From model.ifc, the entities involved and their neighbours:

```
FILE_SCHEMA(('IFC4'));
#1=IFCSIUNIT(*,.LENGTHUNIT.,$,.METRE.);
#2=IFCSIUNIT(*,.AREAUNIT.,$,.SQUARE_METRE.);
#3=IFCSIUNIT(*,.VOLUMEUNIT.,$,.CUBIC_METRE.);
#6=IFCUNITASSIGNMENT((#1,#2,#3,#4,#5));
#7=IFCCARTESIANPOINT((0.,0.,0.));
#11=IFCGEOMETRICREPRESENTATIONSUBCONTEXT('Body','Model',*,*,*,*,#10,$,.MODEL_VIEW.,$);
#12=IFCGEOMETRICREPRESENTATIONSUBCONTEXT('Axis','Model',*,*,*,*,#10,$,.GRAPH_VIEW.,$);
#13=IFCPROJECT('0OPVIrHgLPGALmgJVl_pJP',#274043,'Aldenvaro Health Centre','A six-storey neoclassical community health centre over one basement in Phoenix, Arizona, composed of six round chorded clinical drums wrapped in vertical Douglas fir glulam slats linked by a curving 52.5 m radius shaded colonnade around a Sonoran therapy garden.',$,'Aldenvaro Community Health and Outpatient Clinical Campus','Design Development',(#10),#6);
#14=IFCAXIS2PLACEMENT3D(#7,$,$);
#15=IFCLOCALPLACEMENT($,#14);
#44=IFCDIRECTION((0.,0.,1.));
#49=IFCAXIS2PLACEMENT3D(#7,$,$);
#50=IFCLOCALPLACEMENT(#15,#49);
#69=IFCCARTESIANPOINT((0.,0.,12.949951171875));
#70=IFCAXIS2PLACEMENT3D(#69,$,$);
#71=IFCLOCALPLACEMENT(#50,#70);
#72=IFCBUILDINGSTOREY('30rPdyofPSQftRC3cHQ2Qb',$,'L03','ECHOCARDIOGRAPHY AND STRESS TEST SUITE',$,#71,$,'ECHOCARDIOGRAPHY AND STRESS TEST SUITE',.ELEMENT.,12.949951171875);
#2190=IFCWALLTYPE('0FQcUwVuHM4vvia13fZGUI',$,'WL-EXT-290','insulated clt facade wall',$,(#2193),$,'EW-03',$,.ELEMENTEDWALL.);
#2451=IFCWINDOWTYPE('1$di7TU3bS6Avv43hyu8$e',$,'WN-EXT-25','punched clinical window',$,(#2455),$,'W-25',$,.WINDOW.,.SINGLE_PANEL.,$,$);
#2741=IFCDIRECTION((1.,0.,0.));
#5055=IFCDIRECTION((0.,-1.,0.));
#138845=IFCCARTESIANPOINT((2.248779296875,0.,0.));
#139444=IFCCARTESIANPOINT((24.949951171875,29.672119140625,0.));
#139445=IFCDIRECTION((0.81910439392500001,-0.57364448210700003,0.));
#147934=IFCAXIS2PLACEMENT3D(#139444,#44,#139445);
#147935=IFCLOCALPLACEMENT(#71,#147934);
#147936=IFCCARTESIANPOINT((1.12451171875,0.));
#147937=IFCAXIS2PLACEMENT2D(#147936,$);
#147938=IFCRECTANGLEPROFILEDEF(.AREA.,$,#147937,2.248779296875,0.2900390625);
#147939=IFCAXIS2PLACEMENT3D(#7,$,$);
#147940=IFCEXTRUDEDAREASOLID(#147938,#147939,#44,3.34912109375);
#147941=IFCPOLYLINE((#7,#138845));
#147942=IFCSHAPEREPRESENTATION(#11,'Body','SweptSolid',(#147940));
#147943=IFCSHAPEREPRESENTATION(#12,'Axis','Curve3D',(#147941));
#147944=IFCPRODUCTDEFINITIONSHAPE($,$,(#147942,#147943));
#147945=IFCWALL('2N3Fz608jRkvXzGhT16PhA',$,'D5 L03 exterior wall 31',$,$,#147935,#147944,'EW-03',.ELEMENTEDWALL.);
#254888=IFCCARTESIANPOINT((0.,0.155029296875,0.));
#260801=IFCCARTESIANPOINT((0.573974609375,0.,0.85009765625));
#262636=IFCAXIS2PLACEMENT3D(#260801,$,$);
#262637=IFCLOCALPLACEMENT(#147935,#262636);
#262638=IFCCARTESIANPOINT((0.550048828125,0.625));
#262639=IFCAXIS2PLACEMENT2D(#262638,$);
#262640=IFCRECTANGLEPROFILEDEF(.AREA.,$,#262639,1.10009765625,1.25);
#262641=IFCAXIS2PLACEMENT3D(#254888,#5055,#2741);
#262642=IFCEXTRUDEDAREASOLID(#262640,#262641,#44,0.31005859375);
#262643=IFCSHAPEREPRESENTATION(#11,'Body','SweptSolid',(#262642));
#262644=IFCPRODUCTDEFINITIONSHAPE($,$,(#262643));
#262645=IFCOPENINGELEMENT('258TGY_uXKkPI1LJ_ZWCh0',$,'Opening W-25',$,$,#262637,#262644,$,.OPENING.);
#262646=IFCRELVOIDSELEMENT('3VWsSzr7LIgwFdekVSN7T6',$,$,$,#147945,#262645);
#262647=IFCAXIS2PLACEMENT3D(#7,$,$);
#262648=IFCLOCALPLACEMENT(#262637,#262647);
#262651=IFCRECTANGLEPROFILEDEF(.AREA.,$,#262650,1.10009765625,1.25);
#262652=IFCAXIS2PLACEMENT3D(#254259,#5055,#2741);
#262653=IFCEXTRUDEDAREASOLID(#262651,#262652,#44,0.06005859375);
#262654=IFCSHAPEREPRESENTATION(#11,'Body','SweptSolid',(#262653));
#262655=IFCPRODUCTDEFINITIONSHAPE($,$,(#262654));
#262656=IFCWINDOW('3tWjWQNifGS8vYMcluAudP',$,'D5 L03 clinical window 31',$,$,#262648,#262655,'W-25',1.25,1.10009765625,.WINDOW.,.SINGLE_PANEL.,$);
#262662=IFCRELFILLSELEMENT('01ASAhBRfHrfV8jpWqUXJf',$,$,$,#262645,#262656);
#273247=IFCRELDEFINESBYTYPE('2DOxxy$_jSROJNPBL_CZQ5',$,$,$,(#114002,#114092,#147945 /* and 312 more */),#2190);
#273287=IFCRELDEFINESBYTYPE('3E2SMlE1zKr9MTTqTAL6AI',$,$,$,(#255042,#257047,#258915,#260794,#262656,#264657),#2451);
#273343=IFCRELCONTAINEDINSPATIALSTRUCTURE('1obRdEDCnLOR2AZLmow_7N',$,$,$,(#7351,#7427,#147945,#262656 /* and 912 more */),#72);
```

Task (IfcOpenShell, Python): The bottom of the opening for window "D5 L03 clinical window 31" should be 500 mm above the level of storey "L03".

```python
import numpy as np
import ifcopenshell
import ifcopenshell.api.geometry
import ifcopenshell.geom
import ifcopenshell.util.element
import ifcopenshell.util.placement
import ifcopenshell.util.shape
import ifcopenshell.util.unit

model = ifcopenshell.open("model.ifc")
unit_scale = ifcopenshell.util.unit.calculate_unit_scale(model)

window = model.by_id(262656)
opening = window.FillsVoids[0].RelatingOpeningElement
storey = ifcopenshell.util.element.get_container(window, ifc_class="IfcBuildingStorey")
level = ifcopenshell.util.placement.get_local_placement(storey.ObjectPlacement)[2, 3]

# The opening's origin need not be at the sill, so measure its lowest point.
shape = ifcopenshell.geom.create_shape(ifcopenshell.geom.settings(), opening)
bottom = ifcopenshell.util.shape.get_shape_bottom_elevation(shape, shape.geometry) / unit_scale
dz = level + 0.5 - bottom

shift = np.array([0.0, 0.0, dz])
# The window is placed relative to its opening, so it follows when the opening moves.
matrix = ifcopenshell.util.placement.get_local_placement(opening.ObjectPlacement)
matrix[:3, 3] += shift
ifcopenshell.api.geometry.edit_object_placement(
    model, product=opening, matrix=matrix, is_si=False, should_transform_children=True
)

print(f"moved by {dz * unit_scale:+.3f} m")

model.write("model-out.ifc")
```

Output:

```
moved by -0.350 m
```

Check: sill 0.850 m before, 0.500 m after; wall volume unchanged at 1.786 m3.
